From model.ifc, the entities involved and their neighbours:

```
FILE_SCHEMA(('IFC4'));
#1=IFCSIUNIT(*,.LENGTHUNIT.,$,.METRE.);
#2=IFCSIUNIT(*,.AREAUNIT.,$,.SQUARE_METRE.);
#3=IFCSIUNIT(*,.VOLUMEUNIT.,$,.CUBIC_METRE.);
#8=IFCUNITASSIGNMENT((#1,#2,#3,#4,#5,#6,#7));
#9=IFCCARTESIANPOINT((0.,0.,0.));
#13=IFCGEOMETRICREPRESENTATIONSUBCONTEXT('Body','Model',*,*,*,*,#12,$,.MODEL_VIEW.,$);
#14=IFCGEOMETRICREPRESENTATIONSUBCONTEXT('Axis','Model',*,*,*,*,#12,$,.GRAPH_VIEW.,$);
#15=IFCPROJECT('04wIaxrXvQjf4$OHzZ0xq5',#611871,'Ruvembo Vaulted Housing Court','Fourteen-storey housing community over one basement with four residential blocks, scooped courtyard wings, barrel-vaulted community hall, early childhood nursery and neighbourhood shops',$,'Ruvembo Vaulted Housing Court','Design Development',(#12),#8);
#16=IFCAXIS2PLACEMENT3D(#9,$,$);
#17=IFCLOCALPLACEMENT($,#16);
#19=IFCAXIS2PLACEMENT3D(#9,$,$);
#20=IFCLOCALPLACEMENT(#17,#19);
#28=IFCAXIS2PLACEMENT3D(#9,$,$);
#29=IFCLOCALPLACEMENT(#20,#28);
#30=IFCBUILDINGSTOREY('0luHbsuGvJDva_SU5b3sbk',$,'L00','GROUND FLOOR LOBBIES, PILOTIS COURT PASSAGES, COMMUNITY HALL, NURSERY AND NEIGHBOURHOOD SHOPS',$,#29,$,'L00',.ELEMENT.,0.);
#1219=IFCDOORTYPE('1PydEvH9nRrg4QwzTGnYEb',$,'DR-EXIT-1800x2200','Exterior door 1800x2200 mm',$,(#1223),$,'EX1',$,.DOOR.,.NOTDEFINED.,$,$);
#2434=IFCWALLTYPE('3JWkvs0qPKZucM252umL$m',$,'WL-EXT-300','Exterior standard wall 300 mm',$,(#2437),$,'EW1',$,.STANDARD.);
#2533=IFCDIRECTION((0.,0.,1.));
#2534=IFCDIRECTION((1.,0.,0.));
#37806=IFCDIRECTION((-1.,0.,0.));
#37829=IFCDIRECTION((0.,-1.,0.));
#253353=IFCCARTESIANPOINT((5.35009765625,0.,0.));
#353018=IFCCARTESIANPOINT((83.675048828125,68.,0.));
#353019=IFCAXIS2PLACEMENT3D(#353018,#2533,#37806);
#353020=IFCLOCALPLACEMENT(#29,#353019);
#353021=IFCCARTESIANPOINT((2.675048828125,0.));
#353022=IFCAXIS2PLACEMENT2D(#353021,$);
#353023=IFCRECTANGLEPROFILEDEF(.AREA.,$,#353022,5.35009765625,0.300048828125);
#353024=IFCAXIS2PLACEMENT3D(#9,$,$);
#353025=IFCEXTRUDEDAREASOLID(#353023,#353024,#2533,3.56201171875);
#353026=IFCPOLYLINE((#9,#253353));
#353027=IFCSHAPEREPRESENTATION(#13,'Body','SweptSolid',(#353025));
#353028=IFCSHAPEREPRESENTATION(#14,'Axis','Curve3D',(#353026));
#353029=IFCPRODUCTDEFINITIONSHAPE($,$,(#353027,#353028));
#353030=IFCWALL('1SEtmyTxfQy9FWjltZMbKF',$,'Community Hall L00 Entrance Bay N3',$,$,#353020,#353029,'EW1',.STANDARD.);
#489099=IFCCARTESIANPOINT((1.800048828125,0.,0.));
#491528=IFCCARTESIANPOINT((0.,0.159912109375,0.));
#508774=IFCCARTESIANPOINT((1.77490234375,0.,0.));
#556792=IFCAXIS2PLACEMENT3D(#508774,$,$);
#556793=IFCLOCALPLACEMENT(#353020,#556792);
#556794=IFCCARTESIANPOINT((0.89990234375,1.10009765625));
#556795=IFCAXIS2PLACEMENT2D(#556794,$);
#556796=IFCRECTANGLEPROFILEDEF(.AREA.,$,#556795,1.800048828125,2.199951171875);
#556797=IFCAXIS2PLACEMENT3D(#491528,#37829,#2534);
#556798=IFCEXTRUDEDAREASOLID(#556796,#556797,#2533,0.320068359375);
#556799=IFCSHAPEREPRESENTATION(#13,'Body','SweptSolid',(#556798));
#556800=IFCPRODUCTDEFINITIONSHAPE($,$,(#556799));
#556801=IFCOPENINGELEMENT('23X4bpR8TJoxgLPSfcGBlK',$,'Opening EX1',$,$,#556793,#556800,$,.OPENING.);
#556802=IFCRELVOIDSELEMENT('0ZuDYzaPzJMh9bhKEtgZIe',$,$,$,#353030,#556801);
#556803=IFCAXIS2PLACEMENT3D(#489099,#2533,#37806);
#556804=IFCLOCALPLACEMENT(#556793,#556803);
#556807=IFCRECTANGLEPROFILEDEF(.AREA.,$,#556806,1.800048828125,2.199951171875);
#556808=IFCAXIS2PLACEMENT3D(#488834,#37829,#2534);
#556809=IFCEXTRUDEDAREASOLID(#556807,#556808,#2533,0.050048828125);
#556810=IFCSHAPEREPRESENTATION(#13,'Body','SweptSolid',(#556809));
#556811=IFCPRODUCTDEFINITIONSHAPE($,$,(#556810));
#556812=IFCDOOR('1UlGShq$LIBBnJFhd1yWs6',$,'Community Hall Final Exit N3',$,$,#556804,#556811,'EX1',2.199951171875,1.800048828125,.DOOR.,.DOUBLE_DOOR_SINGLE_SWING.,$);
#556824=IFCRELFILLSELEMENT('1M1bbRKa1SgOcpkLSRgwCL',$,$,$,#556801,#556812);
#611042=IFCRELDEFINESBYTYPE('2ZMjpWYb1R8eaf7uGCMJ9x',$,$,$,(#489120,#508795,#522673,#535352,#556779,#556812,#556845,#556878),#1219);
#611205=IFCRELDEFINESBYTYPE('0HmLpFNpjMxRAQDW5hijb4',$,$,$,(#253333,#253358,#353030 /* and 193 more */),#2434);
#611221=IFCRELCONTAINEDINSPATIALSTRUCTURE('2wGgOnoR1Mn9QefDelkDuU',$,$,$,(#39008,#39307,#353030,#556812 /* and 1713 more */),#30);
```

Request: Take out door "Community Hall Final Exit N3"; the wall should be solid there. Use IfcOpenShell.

```python
import ifcopenshell
import ifcopenshell.api.feature
import ifcopenshell.api.root
import ifcopenshell.geom
import ifcopenshell.util.shape

model = ifcopenshell.open("model.ifc")
settings = ifcopenshell.geom.settings()


def volume(element):
    """Net volume in cubic metres, openings subtracted."""
    shape = ifcopenshell.geom.create_shape(settings, element)
    return ifcopenshell.util.shape.get_volume(shape.geometry)


door = model.by_id(556812)
opening = door.FillsVoids[0].RelatingOpeningElement
wall = opening.VoidsElements[0].RelatingBuildingElement
before = volume(wall)

ifcopenshell.api.root.remove_product(model, product=door)
ifcopenshell.api.feature.remove_feature(model, feature=opening)

after = volume(wall)

print(f"wall volume {before:.3f} -> {after:.3f} m3")

model.write("model-out.ifc")
```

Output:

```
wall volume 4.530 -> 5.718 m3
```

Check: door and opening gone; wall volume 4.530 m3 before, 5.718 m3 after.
